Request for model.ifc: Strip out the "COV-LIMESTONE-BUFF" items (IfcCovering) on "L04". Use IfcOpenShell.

First a look at what the model holds.

```python
import ifcopenshell
import ifcopenshell.util.element

model = ifcopenshell.open("model.ifc")
print(model.schema)
storey = next(s for s in model.by_type("IfcBuildingStorey") if s.Name == "L04")
coverings = [e for e in ifcopenshell.util.element.get_decomposition(storey) if e.is_a("IfcCovering")]
seen = {}
for e in coverings:
    element_type = ifcopenshell.util.element.get_type(e)
    name = element_type.Name if element_type not in (None, e) else None
    seen[name] = seen.get(name, 0) + 1
for name, count in sorted(seen.items(), key=str):
    print(count, "x", name)
```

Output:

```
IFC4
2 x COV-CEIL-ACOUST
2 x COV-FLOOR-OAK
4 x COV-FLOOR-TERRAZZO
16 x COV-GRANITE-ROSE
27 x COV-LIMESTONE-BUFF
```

```python
import ifcopenshell
import ifcopenshell.api.root
import ifcopenshell.util.element

model = ifcopenshell.open("model.ifc")

storey = next(s for s in model.by_type("IfcBuildingStorey") if s.Name == "L04")
coverings = [e for e in ifcopenshell.util.element.get_decomposition(storey) if e.is_a("IfcCovering")]
targets = [e for e in coverings if (t := ifcopenshell.util.element.get_type(e)) not in (None, e) and t.Name == "COV-LIMESTONE-BUFF"]

for e in targets:
    ifcopenshell.api.root.remove_product(model, product=e)
print(len(targets), "removed")

model.write("model_v2.ifc")
```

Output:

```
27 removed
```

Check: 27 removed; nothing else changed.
